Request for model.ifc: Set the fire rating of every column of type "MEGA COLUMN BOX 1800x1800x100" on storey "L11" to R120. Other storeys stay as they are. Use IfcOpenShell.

First a look at what the model holds.

```python
import ifcopenshell
import ifcopenshell.util.element

model = ifcopenshell.open("model.ifc")
print(model.schema)
storey = next(s for s in model.by_type("IfcBuildingStorey") if s.Name == "L11")
columns = [e for e in ifcopenshell.util.element.get_decomposition(storey) if e.is_a("IfcColumn")]
seen = {}
for e in columns:
    element_type = ifcopenshell.util.element.get_type(e)
    key = (element_type.Name if element_type != e and element_type else None, ifcopenshell.util.element.get_pset(e, "Pset_ColumnCommon", "FireRating"))
    seen[key] = seen.get(key, 0) + 1
for (name, value), count in sorted(seen.items(), key=str):
    print(count, "x", name, "|", value)
```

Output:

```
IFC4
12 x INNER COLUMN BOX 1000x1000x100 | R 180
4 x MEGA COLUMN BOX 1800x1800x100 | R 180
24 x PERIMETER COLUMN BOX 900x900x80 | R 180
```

```python
import ifcopenshell
import ifcopenshell.api.pset
import ifcopenshell.util.element

model = ifcopenshell.open("model.ifc")

storey = next(s for s in model.by_type("IfcBuildingStorey") if s.Name == "L11")
columns = [e for e in ifcopenshell.util.element.get_decomposition(storey) if e.is_a("IfcColumn")]

count = 0
for e in columns:
    element_type = ifcopenshell.util.element.get_type(e)
    if element_type in (None, e) or element_type.Name != "MEGA COLUMN BOX 1800x1800x100":
        continue
    # add_pset returns the element's existing set when there is one.
    pset = ifcopenshell.api.pset.add_pset(model, product=e, name="Pset_ColumnCommon")
    ifcopenshell.api.pset.edit_pset(model, pset=pset, properties={"FireRating": "R120"})
    count += 1

print(count, "columns updated")

model.write("model_updated.ifc")
```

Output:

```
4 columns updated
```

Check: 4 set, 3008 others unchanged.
